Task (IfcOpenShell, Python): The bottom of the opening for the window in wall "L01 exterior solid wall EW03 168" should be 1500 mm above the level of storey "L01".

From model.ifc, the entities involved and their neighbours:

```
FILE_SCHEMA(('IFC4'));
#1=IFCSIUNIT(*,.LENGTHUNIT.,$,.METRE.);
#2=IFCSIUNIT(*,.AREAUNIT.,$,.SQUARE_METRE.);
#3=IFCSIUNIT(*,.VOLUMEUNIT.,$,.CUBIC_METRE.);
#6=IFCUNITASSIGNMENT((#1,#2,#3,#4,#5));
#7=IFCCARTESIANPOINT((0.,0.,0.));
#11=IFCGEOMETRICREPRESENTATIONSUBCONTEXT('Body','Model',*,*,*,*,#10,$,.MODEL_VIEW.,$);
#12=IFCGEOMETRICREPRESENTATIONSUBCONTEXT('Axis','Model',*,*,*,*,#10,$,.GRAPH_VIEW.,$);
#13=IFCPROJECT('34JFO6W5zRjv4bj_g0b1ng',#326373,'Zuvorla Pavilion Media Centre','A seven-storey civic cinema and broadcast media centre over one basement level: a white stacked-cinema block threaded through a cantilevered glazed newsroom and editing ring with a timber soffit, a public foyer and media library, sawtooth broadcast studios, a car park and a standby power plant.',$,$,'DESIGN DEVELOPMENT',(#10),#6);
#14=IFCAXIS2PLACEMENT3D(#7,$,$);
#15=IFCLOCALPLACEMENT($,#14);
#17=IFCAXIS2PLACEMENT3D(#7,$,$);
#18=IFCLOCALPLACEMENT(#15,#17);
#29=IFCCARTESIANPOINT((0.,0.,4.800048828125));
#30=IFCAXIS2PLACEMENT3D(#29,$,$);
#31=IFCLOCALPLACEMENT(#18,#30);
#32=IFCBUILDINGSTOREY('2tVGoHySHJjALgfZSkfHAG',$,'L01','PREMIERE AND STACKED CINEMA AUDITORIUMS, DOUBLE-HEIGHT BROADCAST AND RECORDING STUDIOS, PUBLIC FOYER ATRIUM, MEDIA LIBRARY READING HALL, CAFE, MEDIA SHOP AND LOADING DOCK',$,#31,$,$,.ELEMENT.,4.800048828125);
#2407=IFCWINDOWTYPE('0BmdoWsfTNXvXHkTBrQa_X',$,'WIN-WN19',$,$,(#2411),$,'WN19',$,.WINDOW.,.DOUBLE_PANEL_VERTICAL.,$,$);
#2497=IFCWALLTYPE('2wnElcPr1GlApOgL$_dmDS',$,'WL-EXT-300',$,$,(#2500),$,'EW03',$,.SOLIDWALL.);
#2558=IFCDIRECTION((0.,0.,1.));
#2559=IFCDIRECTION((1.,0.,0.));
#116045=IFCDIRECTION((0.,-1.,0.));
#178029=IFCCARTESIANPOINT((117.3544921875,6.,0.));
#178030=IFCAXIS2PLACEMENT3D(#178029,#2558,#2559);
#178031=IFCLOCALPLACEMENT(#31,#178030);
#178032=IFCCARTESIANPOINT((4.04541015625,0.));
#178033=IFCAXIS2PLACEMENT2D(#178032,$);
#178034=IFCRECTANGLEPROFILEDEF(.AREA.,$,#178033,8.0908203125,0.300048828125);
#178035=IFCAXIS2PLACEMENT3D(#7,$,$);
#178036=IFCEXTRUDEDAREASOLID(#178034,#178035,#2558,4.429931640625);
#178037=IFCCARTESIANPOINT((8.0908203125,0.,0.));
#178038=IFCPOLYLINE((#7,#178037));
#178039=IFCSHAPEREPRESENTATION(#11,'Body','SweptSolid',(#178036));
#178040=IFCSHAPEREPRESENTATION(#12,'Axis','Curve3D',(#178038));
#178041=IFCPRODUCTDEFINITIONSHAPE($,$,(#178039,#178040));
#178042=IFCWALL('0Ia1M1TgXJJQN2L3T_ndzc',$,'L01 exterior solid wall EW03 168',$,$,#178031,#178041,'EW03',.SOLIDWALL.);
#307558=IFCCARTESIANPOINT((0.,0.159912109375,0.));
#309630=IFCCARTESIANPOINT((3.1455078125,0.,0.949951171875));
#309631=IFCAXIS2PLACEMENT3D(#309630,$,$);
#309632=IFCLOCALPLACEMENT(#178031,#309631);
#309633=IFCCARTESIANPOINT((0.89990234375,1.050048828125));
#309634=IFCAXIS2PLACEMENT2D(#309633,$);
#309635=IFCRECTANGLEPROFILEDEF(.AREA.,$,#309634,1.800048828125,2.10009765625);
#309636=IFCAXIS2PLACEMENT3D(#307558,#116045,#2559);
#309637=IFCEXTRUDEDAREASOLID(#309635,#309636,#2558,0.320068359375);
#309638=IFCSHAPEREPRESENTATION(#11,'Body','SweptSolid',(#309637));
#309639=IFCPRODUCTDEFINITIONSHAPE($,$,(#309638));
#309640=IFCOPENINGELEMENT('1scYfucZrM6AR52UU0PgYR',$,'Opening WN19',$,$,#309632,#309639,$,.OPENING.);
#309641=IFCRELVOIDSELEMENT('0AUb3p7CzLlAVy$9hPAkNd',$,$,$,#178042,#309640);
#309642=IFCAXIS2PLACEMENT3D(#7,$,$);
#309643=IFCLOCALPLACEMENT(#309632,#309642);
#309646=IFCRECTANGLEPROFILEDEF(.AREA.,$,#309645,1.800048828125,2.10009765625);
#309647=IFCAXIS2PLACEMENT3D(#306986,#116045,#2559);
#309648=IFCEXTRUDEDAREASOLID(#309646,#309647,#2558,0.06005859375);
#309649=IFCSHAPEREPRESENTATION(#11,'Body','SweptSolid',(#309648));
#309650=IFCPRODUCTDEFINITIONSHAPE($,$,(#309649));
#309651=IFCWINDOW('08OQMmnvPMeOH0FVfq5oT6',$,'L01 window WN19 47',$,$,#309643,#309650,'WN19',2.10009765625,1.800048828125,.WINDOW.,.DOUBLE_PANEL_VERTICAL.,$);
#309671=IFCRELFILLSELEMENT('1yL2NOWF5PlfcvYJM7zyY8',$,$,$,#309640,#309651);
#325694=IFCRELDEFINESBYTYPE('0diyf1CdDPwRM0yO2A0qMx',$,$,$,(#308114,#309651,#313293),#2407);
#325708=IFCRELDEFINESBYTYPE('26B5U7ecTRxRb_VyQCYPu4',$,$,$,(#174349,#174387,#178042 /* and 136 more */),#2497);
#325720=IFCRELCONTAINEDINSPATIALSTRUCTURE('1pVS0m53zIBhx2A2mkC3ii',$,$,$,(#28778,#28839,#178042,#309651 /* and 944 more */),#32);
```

```python
import numpy as np
import ifcopenshell
import ifcopenshell.api.geometry
import ifcopenshell.geom
import ifcopenshell.util.element
import ifcopenshell.util.placement
import ifcopenshell.util.shape
import ifcopenshell.util.unit

model = ifcopenshell.open("model.ifc")
unit_scale = ifcopenshell.util.unit.calculate_unit_scale(model)

window = model.by_guid("08OQMmnvPMeOH0FVfq5oT6")
opening = window.FillsVoids[0].RelatingOpeningElement
storey = ifcopenshell.util.element.get_container(window, ifc_class="IfcBuildingStorey")
level = ifcopenshell.util.placement.get_local_placement(storey.ObjectPlacement)[2, 3]

# The opening's origin need not be at the sill, so measure its lowest point.
shape = ifcopenshell.geom.create_shape(ifcopenshell.geom.settings(), opening)
bottom = ifcopenshell.util.shape.get_shape_bottom_elevation(shape, shape.geometry) / unit_scale
dz = level + 1.5 / unit_scale - bottom

shift = np.array([0.0, 0.0, dz])
# The window is placed relative to its opening, so it follows when the opening moves.
matrix = ifcopenshell.util.placement.get_local_placement(opening.ObjectPlacement)
matrix[:3, 3] += shift
ifcopenshell.api.geometry.edit_object_placement(
    model, product=opening, matrix=matrix, is_si=False, should_transform_children=True
)

print(f"moved by {dz * unit_scale:+.3f} m")

model.write("model_updated.ifc")
```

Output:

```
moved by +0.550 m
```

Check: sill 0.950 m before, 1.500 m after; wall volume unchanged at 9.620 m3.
